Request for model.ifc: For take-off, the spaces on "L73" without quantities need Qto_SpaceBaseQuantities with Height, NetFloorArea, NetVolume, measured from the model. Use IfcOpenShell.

First a look at what the model holds.

```python
import ifcopenshell
import ifcopenshell.util.element
import ifcopenshell.util.unit

model = ifcopenshell.open("model.ifc")
print(model.schema)
for unit_type in ("LENGTHUNIT", "AREAUNIT", "VOLUMEUNIT"):
    print(unit_type, ifcopenshell.util.unit.calculate_unit_scale(model, unit_type))
storey = next(s for s in model.by_type("IfcBuildingStorey") if s.Name == "L73")
spaces = [e for e in ifcopenshell.util.element.get_decomposition(storey) if e.is_a("IfcSpace")]
for e in sorted(spaces, key=lambda e: e.id()):
    print(e.id(), e.is_a(), e.Name, list(ifcopenshell.util.element.get_psets(e, qtos_only=True)), sep=" | ")
```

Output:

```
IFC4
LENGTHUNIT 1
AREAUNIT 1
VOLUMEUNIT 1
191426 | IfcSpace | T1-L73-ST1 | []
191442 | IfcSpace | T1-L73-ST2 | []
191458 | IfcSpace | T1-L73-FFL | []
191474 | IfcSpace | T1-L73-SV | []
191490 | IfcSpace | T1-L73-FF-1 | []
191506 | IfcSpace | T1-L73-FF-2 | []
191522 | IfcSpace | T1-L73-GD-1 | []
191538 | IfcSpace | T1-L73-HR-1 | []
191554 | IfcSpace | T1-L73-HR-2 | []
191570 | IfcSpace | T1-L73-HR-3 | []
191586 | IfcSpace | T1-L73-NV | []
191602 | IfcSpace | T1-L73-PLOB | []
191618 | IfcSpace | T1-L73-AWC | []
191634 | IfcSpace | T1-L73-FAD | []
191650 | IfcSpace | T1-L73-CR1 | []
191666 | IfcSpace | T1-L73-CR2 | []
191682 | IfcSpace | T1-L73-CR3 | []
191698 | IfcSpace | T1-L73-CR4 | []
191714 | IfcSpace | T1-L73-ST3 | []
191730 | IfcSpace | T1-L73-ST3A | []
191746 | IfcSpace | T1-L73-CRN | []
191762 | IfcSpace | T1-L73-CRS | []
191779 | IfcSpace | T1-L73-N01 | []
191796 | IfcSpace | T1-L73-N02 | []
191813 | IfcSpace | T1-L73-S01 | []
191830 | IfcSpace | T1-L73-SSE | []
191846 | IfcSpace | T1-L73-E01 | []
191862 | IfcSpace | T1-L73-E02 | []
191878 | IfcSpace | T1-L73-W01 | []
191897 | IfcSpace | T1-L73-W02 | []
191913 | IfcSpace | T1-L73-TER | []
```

```python
import ifcopenshell
import ifcopenshell.api.pset
import ifcopenshell.geom
import ifcopenshell.util.element
import ifcopenshell.util.shape
import ifcopenshell.util.unit

model = ifcopenshell.open("model.ifc")
unit_scale = ifcopenshell.util.unit.calculate_unit_scale(model)
area_scale = ifcopenshell.util.unit.calculate_unit_scale(model, "AREAUNIT")
volume_scale = ifcopenshell.util.unit.calculate_unit_scale(model, "VOLUMEUNIT")
settings = ifcopenshell.geom.settings()

storey = next(s for s in model.by_type("IfcBuildingStorey") if s.Name == "L73")
spaces = [e for e in ifcopenshell.util.element.get_decomposition(storey) if e.is_a("IfcSpace")]

for e in sorted(spaces, key=lambda e: e.id()):
    if ifcopenshell.util.element.get_psets(e, qtos_only=True, should_inherit=False):
        continue
    # Geometry comes back in metres, in the element's own axes.
    shape = ifcopenshell.geom.create_shape(settings, e)
    values = {
        "Height": ifcopenshell.util.shape.get_z(shape.geometry) / unit_scale,
        "NetFloorArea": ifcopenshell.util.shape.get_footprint_area(shape.geometry) / area_scale,
        "NetVolume": ifcopenshell.util.shape.get_volume(shape.geometry) / volume_scale,
    }
    qto = ifcopenshell.api.pset.add_qto(model, product=e, name="Qto_SpaceBaseQuantities")
    ifcopenshell.api.pset.edit_qto(model, qto=qto, properties=values)
    print(e.id(), {k: round(v, 3) for k, v in values.items()})

model.write("model_rev.ifc")
```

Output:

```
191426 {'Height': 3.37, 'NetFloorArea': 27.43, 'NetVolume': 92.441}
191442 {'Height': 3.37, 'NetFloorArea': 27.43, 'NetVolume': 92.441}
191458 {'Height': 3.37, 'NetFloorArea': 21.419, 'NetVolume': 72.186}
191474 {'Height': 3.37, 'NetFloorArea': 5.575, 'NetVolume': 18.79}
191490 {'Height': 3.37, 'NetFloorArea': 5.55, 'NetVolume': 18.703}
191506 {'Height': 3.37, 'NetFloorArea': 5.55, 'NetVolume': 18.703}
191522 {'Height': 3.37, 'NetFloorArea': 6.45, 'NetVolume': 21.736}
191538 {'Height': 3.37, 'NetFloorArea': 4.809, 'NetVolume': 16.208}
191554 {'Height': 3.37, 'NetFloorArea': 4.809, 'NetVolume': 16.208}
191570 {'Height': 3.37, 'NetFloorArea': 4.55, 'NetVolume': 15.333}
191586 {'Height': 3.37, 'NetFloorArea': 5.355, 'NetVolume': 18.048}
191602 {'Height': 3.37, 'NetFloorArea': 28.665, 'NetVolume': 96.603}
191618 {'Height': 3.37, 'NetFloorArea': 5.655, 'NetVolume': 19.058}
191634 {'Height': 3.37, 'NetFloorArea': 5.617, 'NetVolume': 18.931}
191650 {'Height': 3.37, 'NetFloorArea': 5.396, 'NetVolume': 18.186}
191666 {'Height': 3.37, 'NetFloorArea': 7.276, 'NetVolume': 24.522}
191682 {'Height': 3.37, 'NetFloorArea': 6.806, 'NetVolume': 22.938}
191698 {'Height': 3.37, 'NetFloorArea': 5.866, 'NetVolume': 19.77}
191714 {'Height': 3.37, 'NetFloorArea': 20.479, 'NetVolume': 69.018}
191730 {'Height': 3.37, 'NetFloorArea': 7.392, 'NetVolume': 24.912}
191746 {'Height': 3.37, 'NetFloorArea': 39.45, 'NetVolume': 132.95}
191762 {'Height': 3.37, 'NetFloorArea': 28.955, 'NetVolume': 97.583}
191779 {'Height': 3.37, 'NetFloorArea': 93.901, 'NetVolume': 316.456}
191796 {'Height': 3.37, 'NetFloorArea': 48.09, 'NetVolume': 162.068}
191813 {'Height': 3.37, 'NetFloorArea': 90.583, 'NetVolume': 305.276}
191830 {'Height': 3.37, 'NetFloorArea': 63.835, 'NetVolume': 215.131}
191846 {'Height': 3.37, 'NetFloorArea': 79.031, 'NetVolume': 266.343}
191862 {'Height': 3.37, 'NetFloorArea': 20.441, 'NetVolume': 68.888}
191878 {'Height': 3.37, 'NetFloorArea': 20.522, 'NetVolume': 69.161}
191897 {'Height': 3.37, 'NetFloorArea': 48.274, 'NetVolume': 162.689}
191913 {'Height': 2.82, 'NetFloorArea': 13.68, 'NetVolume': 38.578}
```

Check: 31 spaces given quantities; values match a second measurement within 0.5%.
